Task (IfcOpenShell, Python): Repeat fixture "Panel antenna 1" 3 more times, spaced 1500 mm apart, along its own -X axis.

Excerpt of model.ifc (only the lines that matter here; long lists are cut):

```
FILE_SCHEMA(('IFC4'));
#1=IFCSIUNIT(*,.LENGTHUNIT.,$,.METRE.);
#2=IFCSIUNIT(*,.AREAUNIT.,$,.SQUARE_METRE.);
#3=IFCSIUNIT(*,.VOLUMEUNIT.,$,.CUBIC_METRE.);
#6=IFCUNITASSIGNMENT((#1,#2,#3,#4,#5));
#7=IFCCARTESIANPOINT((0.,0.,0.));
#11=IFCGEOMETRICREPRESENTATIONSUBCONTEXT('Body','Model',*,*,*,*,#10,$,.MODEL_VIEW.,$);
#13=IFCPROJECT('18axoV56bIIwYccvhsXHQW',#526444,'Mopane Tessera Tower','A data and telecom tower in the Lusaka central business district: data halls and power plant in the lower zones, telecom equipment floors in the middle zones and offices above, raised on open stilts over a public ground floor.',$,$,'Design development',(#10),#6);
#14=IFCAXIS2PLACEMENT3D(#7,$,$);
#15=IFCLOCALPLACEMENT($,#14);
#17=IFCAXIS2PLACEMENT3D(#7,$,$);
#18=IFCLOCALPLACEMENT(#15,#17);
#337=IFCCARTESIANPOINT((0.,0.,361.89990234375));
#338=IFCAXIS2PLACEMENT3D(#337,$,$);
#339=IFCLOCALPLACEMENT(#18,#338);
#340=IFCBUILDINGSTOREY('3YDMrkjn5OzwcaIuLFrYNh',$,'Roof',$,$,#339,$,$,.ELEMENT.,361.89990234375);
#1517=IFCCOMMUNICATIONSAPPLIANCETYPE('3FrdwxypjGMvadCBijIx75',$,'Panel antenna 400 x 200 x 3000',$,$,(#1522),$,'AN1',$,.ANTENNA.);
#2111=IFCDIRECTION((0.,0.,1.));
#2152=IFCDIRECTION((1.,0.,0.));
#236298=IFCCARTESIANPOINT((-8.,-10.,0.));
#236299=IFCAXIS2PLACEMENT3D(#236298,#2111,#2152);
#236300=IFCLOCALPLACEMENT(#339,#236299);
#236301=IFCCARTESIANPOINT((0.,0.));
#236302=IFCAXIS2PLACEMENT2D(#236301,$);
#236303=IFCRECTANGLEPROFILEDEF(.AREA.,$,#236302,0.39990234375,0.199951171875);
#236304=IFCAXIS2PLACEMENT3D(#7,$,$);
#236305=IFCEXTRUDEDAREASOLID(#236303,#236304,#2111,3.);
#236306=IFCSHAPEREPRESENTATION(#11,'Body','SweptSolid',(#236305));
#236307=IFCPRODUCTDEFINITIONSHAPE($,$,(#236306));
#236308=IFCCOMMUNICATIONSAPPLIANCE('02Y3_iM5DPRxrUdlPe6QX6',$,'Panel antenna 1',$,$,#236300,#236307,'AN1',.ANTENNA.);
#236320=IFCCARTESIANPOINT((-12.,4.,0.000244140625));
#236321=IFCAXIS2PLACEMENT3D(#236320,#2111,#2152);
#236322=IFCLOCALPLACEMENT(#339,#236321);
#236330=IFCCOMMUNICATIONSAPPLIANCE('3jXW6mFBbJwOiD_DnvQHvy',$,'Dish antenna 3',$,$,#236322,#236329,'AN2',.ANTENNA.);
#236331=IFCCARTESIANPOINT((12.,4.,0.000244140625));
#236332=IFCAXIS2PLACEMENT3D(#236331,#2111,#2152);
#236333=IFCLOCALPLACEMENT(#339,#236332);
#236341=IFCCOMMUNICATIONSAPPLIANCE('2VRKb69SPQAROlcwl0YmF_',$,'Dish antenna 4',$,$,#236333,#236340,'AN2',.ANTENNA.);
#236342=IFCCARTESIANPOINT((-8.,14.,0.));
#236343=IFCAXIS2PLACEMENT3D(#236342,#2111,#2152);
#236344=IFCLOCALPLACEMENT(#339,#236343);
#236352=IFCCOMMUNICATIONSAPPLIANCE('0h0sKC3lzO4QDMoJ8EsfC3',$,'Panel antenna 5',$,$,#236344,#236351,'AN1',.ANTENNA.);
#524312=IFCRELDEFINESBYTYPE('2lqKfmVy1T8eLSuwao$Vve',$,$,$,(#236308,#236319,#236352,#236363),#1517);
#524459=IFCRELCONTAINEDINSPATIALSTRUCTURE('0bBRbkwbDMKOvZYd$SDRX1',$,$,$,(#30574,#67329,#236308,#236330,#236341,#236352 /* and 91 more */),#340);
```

```python
import ifcopenshell
import ifcopenshell.api.geometry
import ifcopenshell.api.root
import ifcopenshell.util.element
import ifcopenshell.util.placement
import ifcopenshell.util.unit

model = ifcopenshell.open("model.ifc")
unit_scale = ifcopenshell.util.unit.calculate_unit_scale(model)

source = model.by_guid("02Y3_iM5DPRxrUdlPe6QX6")
base = ifcopenshell.util.placement.get_local_placement(source.ObjectPlacement)
step = -base[:3, 0] * 1.5 / unit_scale

for i in range(1, 4):
    copy = ifcopenshell.api.root.copy_class(model, product=source)
    copy.Representation = ifcopenshell.util.element.copy_deep(
        model, source.Representation, exclude=["IfcGeometricRepresentationContext", "IfcRepresentationMap"]
    )
    copy.Tag = None
    matrix = base.copy()
    matrix[:3, 3] += i * step
    print("added at", matrix[:3, 3].round(3) + 0.0)
    ifcopenshell.api.geometry.edit_object_placement(model, product=copy, matrix=matrix, is_si=False)

model.write("model_v2.ifc")
```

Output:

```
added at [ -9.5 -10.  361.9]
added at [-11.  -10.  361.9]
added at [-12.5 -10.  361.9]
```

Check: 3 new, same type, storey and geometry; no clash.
